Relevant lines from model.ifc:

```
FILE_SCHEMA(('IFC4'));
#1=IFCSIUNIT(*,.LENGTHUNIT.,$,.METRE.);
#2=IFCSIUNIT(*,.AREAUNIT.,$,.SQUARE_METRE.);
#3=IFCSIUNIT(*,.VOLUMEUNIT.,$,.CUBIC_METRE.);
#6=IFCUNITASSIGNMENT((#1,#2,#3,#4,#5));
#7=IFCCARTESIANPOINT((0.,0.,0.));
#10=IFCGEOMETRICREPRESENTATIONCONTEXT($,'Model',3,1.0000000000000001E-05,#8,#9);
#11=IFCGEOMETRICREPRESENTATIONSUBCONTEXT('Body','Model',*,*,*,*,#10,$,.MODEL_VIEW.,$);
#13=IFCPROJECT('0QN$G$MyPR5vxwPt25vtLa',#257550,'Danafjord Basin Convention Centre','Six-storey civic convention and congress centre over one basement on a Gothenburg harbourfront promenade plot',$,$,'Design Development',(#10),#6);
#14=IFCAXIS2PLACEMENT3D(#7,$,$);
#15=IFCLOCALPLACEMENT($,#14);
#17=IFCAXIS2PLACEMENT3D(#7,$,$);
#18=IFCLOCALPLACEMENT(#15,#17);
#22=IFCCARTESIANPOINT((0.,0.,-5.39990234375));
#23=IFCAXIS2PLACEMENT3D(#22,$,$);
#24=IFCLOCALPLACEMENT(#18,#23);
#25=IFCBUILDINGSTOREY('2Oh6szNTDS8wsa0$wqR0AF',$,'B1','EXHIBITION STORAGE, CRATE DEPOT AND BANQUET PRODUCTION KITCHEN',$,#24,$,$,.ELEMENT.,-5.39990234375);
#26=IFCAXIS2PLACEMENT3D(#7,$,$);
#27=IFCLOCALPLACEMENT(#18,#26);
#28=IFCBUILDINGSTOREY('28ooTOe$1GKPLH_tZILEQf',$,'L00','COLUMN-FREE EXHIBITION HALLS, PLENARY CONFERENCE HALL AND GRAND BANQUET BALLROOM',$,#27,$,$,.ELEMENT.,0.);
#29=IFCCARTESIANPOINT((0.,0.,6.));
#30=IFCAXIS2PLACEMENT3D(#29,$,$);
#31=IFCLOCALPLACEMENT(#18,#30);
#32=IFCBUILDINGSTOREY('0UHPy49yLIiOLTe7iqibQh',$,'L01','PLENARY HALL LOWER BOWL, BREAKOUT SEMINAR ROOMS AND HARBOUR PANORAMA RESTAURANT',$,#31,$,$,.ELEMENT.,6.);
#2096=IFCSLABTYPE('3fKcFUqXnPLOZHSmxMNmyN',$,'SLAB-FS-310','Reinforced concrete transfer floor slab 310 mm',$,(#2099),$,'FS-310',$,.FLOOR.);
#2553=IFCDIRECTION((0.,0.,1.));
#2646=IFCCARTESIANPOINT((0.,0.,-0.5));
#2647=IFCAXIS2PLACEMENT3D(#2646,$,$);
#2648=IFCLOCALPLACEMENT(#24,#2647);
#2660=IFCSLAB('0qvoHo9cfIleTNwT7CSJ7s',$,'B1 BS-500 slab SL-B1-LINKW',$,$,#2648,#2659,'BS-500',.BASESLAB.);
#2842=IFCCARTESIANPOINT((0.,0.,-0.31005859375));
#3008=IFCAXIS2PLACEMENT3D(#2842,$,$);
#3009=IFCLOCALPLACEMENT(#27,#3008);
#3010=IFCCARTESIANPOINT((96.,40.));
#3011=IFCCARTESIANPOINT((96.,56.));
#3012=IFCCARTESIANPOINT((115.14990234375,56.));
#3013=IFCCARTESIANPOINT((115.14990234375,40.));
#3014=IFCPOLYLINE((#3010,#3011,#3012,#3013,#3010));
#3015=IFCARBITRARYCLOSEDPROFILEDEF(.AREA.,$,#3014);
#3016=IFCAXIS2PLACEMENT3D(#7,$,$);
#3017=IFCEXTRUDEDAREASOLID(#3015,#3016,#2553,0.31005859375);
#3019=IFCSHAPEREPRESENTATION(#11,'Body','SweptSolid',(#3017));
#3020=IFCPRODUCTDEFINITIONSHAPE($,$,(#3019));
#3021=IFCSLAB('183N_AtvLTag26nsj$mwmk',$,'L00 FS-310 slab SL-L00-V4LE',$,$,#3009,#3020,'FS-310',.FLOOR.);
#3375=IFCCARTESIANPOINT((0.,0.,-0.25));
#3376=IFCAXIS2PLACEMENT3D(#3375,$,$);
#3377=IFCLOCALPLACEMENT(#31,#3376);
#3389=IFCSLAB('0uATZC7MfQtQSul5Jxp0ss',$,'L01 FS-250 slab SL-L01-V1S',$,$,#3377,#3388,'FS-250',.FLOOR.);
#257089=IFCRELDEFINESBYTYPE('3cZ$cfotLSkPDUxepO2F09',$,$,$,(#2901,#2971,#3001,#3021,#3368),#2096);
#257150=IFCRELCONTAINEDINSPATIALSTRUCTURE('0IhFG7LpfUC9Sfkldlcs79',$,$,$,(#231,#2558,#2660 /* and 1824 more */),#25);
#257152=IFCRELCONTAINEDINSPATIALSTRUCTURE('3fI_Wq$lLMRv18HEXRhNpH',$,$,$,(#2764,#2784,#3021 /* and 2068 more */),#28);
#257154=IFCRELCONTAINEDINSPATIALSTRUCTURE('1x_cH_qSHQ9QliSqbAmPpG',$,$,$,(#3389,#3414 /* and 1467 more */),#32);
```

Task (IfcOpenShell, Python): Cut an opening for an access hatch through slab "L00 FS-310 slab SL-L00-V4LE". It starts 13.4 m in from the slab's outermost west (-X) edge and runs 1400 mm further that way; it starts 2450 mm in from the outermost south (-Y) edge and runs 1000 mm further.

```python
import numpy as np
import ifcopenshell
import ifcopenshell.api.feature
import ifcopenshell.api.geometry
import ifcopenshell.api.root
import ifcopenshell.geom
import ifcopenshell.util.placement
import ifcopenshell.util.representation
import ifcopenshell.util.shape
import ifcopenshell.util.unit

model = ifcopenshell.open("model.ifc")
unit_scale = ifcopenshell.util.unit.calculate_unit_scale(model)
settings = ifcopenshell.geom.settings()


def volume(element):
    """Net volume in cubic metres, openings subtracted."""
    shape = ifcopenshell.geom.create_shape(settings, element)
    return ifcopenshell.util.shape.get_volume(shape.geometry)


slab = model.by_id(3021)
before = volume(slab)

# Extent in the slab's own axes, in metres. The edges named are its -X and -Y sides.
slab_shape = ifcopenshell.geom.create_shape(settings, slab)
vertices = ifcopenshell.util.shape.get_vertices(slab_shape.geometry)
x_min, y_min, bottom = vertices.min(axis=0)
top = vertices[:, 2].max()

opening = ifcopenshell.api.root.create_entity(model, ifc_class="IfcOpeningElement", name="Access hatch opening", predefined_type="OPENING")
context = ifcopenshell.util.representation.get_context(model, "Model", "Body", "MODEL_VIEW")
width, depth = 1.4, 1
outline = [(0.0, 0.0), (width, 0.0), (width, depth), (0.0, depth), (0.0, 0.0)]
# Overshoot both faces by 50 mm so the cut is clean.
shape = ifcopenshell.api.geometry.add_slab_representation(
    model, context=context, depth=top - bottom + 0.1, polyline=outline
)
ifcopenshell.api.geometry.assign_representation(model, product=opening, representation=shape)

matrix = ifcopenshell.util.placement.get_local_placement(slab.ObjectPlacement)
matrix[:, 3] = matrix @ np.append(np.array([x_min + 13.4, y_min + 2.45, bottom - 0.05]) / unit_scale, 1.0)
ifcopenshell.api.geometry.edit_object_placement(model, product=opening, matrix=matrix, is_si=False)
ifcopenshell.api.feature.add_feature(model, feature=opening, element=slab)

after = volume(slab)

print(f"slab volume {before:.3f} -> {after:.3f} m3")

model.write("model_edited.ifc")
```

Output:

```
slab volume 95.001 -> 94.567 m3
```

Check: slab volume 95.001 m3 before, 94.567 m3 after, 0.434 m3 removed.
